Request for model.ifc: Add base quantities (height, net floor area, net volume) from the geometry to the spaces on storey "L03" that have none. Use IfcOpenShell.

First a look at what the model holds.

```python
import ifcopenshell
import ifcopenshell.util.element
import ifcopenshell.util.unit

model = ifcopenshell.open("model.ifc")
print(model.schema)
for unit_type in ("LENGTHUNIT", "AREAUNIT", "VOLUMEUNIT"):
    print(unit_type, ifcopenshell.util.unit.calculate_unit_scale(model, unit_type))
storey = next(s for s in model.by_type("IfcBuildingStorey") if s.Name == "L03")
spaces = [e for e in ifcopenshell.util.element.get_decomposition(storey) if e.is_a("IfcSpace")]
for e in sorted(spaces, key=lambda e: e.id()):
    print(e.id(), e.is_a(), e.Name, list(ifcopenshell.util.element.get_psets(e, qtos_only=True)), sep=" | ")
```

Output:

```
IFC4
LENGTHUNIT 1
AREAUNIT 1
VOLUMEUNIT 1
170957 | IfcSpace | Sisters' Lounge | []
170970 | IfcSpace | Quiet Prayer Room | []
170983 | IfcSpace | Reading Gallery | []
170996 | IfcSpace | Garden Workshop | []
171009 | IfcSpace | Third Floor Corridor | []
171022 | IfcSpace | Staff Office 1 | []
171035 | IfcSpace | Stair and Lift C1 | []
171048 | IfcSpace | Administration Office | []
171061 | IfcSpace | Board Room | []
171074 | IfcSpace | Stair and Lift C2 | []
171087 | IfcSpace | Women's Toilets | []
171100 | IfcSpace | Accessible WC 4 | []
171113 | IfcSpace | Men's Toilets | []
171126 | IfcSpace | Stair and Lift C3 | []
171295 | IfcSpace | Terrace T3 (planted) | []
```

```python
import ifcopenshell
import ifcopenshell.api.pset
import ifcopenshell.geom
import ifcopenshell.util.element
import ifcopenshell.util.shape
import ifcopenshell.util.unit

model = ifcopenshell.open("model.ifc")
unit_scale = ifcopenshell.util.unit.calculate_unit_scale(model)
area_scale = ifcopenshell.util.unit.calculate_unit_scale(model, "AREAUNIT")
volume_scale = ifcopenshell.util.unit.calculate_unit_scale(model, "VOLUMEUNIT")
settings = ifcopenshell.geom.settings()

storey = next(s for s in model.by_type("IfcBuildingStorey") if s.Name == "L03")
spaces = [e for e in ifcopenshell.util.element.get_decomposition(storey) if e.is_a("IfcSpace")]

for e in sorted(spaces, key=lambda e: e.id()):
    if ifcopenshell.util.element.get_psets(e, qtos_only=True, should_inherit=False):
        continue
    # Geometry comes back in metres, in the element's own axes.
    shape = ifcopenshell.geom.create_shape(settings, e)
    values = {
        "Height": ifcopenshell.util.shape.get_z(shape.geometry) / unit_scale,
        "NetFloorArea": ifcopenshell.util.shape.get_footprint_area(shape.geometry) / area_scale,
        "NetVolume": ifcopenshell.util.shape.get_volume(shape.geometry) / volume_scale,
    }
    qto = ifcopenshell.api.pset.add_qto(model, product=e, name="Qto_SpaceBaseQuantities")
    ifcopenshell.api.pset.edit_qto(model, qto=qto, properties=values)
    print(e.id(), {k: round(v, 3) for k, v in values.items()})

model.write("model-out.ifc")
```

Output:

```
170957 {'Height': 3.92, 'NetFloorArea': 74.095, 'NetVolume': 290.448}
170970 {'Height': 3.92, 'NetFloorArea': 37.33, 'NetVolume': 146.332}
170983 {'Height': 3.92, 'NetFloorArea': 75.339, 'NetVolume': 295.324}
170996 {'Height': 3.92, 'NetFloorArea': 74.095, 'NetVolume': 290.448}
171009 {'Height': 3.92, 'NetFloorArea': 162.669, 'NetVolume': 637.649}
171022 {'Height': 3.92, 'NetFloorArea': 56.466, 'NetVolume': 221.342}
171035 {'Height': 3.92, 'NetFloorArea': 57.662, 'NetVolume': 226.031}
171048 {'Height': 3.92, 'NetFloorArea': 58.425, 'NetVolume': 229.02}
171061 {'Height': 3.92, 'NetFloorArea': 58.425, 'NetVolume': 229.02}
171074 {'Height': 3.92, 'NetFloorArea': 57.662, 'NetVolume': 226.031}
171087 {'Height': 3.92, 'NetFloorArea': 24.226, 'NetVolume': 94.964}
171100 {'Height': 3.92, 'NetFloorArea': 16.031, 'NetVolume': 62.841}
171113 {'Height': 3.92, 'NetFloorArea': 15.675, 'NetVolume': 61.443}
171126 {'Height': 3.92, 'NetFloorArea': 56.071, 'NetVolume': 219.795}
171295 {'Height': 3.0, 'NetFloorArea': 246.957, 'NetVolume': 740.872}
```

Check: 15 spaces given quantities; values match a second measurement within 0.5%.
